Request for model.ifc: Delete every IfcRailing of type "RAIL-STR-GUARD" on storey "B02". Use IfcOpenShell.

First a look at what the model holds.

```python
import ifcopenshell
import ifcopenshell.util.element

model = ifcopenshell.open("model.ifc")
print(model.schema)
storey = next(s for s in model.by_type("IfcBuildingStorey") if s.Name == "B02")
railings = [e for e in ifcopenshell.util.element.get_decomposition(storey) if e.is_a("IfcRailing")]
seen = {}
for e in railings:
    element_type = ifcopenshell.util.element.get_type(e)
    name = element_type.Name if element_type not in (None, e) else None
    seen[name] = seen.get(name, 0) + 1
for name, count in sorted(seen.items(), key=str):
    print(count, "x", name)
```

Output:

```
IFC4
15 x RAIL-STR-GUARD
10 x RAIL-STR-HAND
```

```python
import ifcopenshell
import ifcopenshell.api.root
import ifcopenshell.util.element

model = ifcopenshell.open("model.ifc")

storey = next(s for s in model.by_type("IfcBuildingStorey") if s.Name == "B02")
railings = [e for e in ifcopenshell.util.element.get_decomposition(storey) if e.is_a("IfcRailing")]
targets = [e for e in railings if (t := ifcopenshell.util.element.get_type(e)) not in (None, e) and t.Name == "RAIL-STR-GUARD"]

for e in targets:
    ifcopenshell.api.root.remove_product(model, product=e)
print(len(targets), "removed")

model.write("model_v2.ifc")
```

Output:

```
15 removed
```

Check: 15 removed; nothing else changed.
